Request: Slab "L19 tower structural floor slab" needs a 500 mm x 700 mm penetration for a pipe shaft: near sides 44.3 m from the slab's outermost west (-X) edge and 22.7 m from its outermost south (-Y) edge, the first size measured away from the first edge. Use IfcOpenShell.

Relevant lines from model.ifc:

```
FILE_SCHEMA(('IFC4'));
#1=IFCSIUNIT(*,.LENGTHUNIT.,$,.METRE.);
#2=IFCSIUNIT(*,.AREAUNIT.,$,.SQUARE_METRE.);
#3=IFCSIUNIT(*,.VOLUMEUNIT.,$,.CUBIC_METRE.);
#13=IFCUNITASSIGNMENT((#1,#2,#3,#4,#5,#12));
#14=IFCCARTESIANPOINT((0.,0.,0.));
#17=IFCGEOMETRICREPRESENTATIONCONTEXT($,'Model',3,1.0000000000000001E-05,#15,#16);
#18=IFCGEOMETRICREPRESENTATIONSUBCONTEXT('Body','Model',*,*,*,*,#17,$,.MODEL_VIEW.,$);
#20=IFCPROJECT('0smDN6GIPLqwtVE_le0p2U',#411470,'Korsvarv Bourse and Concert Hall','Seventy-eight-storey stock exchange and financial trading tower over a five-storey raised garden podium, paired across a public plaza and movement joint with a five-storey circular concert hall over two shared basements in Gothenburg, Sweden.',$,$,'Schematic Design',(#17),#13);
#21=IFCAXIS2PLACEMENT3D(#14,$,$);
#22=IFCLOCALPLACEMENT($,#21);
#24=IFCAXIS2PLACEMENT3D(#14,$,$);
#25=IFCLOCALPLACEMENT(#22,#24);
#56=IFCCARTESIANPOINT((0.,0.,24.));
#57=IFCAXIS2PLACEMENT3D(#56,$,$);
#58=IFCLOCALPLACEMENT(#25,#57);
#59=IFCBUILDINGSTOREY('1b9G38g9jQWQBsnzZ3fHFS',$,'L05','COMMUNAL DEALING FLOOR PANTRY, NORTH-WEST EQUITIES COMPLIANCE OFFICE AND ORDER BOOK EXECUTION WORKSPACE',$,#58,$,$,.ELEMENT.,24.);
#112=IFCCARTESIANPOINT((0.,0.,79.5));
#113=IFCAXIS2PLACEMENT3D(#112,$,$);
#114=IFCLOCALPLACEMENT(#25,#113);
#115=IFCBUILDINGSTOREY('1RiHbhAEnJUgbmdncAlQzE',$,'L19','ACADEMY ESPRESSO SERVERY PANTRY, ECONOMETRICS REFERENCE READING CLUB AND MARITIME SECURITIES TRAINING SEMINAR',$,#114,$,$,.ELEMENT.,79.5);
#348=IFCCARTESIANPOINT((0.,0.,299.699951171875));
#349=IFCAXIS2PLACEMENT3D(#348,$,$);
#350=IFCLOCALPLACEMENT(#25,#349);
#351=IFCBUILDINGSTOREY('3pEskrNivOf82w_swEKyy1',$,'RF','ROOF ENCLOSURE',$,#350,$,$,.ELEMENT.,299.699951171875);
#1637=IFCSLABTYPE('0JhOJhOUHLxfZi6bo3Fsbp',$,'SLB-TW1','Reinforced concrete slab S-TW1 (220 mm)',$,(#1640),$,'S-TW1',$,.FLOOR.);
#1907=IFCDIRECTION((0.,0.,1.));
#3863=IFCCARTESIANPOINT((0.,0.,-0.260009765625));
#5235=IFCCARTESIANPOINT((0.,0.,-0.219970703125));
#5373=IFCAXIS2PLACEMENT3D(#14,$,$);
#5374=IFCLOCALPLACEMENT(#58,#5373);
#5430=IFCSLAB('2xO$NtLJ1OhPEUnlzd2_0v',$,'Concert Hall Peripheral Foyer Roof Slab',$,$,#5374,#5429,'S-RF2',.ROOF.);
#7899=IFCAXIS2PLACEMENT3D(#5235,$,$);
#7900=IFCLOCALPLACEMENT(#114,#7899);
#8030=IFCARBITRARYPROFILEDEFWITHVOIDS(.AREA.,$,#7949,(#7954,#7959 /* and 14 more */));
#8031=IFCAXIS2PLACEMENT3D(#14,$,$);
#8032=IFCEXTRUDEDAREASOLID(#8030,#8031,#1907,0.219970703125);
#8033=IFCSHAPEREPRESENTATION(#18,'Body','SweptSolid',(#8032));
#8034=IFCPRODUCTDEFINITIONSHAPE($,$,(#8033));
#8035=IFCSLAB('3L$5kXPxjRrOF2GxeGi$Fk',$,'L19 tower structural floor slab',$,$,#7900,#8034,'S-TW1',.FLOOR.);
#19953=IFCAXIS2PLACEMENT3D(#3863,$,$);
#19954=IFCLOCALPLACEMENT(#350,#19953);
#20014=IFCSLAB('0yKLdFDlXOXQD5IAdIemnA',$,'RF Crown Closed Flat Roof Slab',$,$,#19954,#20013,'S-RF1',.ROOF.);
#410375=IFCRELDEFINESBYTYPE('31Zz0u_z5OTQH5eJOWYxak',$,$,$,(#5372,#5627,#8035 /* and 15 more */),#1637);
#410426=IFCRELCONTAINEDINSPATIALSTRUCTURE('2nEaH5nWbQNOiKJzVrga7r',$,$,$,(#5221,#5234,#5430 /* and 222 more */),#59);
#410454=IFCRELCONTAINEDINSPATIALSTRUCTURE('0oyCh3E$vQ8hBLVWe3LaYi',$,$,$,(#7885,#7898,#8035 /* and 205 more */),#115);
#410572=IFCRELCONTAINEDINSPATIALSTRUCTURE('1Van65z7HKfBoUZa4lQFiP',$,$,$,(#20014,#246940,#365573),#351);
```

```python
import numpy as np
import ifcopenshell
import ifcopenshell.api.feature
import ifcopenshell.api.geometry
import ifcopenshell.api.root
import ifcopenshell.geom
import ifcopenshell.util.placement
import ifcopenshell.util.representation
import ifcopenshell.util.shape
import ifcopenshell.util.unit

model = ifcopenshell.open("model.ifc")
unit_scale = ifcopenshell.util.unit.calculate_unit_scale(model)
settings = ifcopenshell.geom.settings()


def volume(element):
    """Net volume in cubic metres, openings subtracted."""
    shape = ifcopenshell.geom.create_shape(settings, element)
    return ifcopenshell.util.shape.get_volume(shape.geometry)


slab = model.by_id(8035)
before = volume(slab)

# Extent in the slab's own axes, in metres. The edges named are its -X and -Y sides.
slab_shape = ifcopenshell.geom.create_shape(settings, slab)
vertices = ifcopenshell.util.shape.get_vertices(slab_shape.geometry)
x_min, y_min, bottom = vertices.min(axis=0)
top = vertices[:, 2].max()

opening = ifcopenshell.api.root.create_entity(model, ifc_class="IfcOpeningElement", name="Pipe shaft opening", predefined_type="OPENING")
context = ifcopenshell.util.representation.get_context(model, "Model", "Body", "MODEL_VIEW")
width, depth = 0.5, 0.7
outline = [(0.0, 0.0), (width, 0.0), (width, depth), (0.0, depth), (0.0, 0.0)]
# Overshoot both faces by 50 mm so the cut is clean.
shape = ifcopenshell.api.geometry.add_slab_representation(
    model, context=context, depth=top - bottom + 0.1, polyline=outline
)
ifcopenshell.api.geometry.assign_representation(model, product=opening, representation=shape)

matrix = ifcopenshell.util.placement.get_local_placement(slab.ObjectPlacement)
matrix[:, 3] = matrix @ np.append(np.array([x_min + 44.3, y_min + 22.7, bottom - 0.05]) / unit_scale, 1.0)
ifcopenshell.api.geometry.edit_object_placement(model, product=opening, matrix=matrix, is_si=False)
ifcopenshell.api.feature.add_feature(model, feature=opening, element=slab)

after = volume(slab)

print(f"slab volume {before:.3f} -> {after:.3f} m3")

model.write("model_rev.ifc")
```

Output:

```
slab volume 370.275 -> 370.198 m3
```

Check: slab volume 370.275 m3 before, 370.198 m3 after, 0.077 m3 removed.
